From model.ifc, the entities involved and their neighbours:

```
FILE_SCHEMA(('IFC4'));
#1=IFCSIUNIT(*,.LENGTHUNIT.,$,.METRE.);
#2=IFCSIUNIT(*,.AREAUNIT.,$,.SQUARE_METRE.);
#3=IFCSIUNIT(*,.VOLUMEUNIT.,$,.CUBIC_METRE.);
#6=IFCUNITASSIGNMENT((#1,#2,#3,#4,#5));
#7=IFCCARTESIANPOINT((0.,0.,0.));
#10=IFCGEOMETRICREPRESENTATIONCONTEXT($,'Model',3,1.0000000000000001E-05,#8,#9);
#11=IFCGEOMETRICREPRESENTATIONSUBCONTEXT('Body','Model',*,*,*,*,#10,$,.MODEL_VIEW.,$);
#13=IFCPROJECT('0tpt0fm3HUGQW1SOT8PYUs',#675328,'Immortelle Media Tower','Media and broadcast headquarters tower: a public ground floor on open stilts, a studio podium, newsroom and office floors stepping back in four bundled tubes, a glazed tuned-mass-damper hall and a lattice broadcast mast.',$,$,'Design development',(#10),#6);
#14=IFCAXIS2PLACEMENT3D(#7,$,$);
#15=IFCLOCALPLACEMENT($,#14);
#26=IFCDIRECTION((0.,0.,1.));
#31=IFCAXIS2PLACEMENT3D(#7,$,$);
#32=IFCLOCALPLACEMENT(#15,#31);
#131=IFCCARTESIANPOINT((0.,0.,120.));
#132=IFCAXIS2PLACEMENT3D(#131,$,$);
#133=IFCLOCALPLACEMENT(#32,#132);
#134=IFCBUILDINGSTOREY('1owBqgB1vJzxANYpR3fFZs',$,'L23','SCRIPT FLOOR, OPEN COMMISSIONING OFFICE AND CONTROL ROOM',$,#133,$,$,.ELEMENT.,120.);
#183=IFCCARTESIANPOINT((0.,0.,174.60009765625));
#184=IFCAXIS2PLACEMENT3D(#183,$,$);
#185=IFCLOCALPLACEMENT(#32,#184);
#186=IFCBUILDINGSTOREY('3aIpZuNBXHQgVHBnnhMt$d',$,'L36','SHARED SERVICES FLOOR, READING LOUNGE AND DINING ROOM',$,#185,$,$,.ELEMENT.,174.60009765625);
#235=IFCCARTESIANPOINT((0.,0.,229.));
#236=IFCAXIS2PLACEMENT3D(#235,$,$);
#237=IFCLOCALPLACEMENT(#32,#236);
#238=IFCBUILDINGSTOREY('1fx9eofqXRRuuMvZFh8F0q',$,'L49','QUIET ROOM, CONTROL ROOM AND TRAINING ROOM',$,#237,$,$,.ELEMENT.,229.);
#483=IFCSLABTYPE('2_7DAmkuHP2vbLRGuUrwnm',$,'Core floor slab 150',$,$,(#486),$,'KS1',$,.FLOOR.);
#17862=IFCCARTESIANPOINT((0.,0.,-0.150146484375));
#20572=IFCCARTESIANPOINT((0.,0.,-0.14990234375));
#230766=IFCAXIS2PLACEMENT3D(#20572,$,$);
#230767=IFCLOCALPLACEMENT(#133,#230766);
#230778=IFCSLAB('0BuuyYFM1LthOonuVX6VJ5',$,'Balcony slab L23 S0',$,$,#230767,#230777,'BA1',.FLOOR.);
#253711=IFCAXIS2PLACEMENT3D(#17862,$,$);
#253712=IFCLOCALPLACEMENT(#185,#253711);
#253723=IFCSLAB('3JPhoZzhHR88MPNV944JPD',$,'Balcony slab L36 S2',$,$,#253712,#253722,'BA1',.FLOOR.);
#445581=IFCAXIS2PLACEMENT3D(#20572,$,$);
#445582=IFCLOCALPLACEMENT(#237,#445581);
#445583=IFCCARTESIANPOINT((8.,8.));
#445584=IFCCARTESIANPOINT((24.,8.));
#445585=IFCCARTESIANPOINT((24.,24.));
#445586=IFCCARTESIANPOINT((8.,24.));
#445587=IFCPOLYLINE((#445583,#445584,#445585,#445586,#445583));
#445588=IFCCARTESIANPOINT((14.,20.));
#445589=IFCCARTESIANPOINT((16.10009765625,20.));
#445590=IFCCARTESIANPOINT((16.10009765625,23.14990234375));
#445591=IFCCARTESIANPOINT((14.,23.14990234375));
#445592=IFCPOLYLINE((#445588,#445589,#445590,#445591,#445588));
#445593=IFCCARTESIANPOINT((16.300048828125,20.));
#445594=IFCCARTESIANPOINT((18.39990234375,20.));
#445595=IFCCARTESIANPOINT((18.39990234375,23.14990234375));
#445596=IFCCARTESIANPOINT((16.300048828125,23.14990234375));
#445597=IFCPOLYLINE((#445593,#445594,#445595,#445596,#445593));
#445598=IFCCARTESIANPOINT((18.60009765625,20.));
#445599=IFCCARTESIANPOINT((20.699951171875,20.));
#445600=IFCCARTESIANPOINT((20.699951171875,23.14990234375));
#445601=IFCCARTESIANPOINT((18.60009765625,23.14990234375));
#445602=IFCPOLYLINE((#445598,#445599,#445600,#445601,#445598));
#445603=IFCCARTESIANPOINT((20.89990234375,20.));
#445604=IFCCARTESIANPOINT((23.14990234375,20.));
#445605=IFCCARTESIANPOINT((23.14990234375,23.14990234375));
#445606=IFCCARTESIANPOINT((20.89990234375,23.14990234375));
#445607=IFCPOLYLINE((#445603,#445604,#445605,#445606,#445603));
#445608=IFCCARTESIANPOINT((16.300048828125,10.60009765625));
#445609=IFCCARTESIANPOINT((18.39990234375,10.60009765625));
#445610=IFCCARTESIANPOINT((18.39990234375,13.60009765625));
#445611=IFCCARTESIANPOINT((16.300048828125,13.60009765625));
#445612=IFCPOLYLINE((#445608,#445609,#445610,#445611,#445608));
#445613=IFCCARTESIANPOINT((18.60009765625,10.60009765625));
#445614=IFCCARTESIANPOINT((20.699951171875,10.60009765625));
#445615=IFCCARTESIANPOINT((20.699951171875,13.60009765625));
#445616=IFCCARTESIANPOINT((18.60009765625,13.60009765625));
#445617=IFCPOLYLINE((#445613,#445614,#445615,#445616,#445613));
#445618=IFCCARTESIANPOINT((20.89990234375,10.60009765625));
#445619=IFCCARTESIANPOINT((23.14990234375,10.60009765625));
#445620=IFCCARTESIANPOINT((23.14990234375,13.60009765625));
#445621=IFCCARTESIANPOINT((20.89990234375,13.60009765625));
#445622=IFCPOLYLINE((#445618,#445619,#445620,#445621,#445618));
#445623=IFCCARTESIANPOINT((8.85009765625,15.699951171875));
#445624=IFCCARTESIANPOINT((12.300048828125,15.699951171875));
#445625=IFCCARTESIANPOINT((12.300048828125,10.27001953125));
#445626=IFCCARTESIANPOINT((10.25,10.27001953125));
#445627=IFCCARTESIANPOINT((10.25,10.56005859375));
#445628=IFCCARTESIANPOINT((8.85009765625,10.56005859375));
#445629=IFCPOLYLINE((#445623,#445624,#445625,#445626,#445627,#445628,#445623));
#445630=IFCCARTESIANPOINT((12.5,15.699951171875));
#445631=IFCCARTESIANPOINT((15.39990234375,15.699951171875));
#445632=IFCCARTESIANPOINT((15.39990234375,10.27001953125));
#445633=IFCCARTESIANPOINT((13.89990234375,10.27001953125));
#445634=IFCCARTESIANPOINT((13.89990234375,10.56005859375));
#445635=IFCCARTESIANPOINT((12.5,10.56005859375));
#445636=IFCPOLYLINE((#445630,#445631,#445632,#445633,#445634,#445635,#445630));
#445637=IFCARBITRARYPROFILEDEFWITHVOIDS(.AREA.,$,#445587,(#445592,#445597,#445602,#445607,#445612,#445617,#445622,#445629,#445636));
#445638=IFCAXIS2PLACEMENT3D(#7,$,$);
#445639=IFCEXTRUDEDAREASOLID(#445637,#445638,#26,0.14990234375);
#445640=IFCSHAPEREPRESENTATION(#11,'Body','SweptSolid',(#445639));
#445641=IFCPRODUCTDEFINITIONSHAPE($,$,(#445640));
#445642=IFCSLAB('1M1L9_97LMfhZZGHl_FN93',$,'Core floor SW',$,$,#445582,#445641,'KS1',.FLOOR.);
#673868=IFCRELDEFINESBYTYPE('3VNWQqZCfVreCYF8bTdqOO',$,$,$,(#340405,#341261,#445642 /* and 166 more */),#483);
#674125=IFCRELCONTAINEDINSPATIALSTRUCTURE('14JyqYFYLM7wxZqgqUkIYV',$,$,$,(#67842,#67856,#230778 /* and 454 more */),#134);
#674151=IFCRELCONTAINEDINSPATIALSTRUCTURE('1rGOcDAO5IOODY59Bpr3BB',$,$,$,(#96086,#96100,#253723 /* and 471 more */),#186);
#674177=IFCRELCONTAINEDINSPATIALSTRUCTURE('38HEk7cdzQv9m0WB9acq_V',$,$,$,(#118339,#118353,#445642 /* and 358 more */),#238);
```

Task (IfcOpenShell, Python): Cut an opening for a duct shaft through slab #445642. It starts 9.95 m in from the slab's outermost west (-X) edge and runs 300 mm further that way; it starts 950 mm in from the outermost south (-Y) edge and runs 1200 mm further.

```python
import numpy as np
import ifcopenshell
import ifcopenshell.api.feature
import ifcopenshell.api.geometry
import ifcopenshell.api.root
import ifcopenshell.geom
import ifcopenshell.util.placement
import ifcopenshell.util.representation
import ifcopenshell.util.shape
import ifcopenshell.util.unit

model = ifcopenshell.open("model.ifc")
unit_scale = ifcopenshell.util.unit.calculate_unit_scale(model)
settings = ifcopenshell.geom.settings()


def volume(element):
    """Net volume in cubic metres, openings subtracted."""
    shape = ifcopenshell.geom.create_shape(settings, element)
    return ifcopenshell.util.shape.get_volume(shape.geometry)


slab = model.by_guid("1M1L9_97LMfhZZGHl_FN93")
before = volume(slab)

# Extent in the slab's own axes, in metres. The edges named are its -X and -Y sides.
slab_shape = ifcopenshell.geom.create_shape(settings, slab)
vertices = ifcopenshell.util.shape.get_vertices(slab_shape.geometry)
x_min, y_min, bottom = vertices.min(axis=0)
top = vertices[:, 2].max()

opening = ifcopenshell.api.root.create_entity(model, ifc_class="IfcOpeningElement", name="Duct shaft opening", predefined_type="OPENING")
context = ifcopenshell.util.representation.get_context(model, "Model", "Body", "MODEL_VIEW")
width, depth = 0.3, 1.2
outline = [(0.0, 0.0), (width, 0.0), (width, depth), (0.0, depth), (0.0, 0.0)]
# Overshoot both faces by 50 mm so the cut is clean.
shape = ifcopenshell.api.geometry.add_slab_representation(
    model, context=context, depth=top - bottom + 0.1, polyline=outline
)
ifcopenshell.api.geometry.assign_representation(model, product=opening, representation=shape)

matrix = ifcopenshell.util.placement.get_local_placement(slab.ObjectPlacement)
matrix[:, 3] = matrix @ np.append(np.array([x_min + 9.95, y_min + 0.95, bottom - 0.05]) / unit_scale, 1.0)
ifcopenshell.api.geometry.edit_object_placement(model, product=opening, matrix=matrix, is_si=False)
ifcopenshell.api.feature.add_feature(model, feature=opening, element=slab)

after = volume(slab)

print(f"slab volume {before:.3f} -> {after:.3f} m3")

model.write("model_edited.ifc")
```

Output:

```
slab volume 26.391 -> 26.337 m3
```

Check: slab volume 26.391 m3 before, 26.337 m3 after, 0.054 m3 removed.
